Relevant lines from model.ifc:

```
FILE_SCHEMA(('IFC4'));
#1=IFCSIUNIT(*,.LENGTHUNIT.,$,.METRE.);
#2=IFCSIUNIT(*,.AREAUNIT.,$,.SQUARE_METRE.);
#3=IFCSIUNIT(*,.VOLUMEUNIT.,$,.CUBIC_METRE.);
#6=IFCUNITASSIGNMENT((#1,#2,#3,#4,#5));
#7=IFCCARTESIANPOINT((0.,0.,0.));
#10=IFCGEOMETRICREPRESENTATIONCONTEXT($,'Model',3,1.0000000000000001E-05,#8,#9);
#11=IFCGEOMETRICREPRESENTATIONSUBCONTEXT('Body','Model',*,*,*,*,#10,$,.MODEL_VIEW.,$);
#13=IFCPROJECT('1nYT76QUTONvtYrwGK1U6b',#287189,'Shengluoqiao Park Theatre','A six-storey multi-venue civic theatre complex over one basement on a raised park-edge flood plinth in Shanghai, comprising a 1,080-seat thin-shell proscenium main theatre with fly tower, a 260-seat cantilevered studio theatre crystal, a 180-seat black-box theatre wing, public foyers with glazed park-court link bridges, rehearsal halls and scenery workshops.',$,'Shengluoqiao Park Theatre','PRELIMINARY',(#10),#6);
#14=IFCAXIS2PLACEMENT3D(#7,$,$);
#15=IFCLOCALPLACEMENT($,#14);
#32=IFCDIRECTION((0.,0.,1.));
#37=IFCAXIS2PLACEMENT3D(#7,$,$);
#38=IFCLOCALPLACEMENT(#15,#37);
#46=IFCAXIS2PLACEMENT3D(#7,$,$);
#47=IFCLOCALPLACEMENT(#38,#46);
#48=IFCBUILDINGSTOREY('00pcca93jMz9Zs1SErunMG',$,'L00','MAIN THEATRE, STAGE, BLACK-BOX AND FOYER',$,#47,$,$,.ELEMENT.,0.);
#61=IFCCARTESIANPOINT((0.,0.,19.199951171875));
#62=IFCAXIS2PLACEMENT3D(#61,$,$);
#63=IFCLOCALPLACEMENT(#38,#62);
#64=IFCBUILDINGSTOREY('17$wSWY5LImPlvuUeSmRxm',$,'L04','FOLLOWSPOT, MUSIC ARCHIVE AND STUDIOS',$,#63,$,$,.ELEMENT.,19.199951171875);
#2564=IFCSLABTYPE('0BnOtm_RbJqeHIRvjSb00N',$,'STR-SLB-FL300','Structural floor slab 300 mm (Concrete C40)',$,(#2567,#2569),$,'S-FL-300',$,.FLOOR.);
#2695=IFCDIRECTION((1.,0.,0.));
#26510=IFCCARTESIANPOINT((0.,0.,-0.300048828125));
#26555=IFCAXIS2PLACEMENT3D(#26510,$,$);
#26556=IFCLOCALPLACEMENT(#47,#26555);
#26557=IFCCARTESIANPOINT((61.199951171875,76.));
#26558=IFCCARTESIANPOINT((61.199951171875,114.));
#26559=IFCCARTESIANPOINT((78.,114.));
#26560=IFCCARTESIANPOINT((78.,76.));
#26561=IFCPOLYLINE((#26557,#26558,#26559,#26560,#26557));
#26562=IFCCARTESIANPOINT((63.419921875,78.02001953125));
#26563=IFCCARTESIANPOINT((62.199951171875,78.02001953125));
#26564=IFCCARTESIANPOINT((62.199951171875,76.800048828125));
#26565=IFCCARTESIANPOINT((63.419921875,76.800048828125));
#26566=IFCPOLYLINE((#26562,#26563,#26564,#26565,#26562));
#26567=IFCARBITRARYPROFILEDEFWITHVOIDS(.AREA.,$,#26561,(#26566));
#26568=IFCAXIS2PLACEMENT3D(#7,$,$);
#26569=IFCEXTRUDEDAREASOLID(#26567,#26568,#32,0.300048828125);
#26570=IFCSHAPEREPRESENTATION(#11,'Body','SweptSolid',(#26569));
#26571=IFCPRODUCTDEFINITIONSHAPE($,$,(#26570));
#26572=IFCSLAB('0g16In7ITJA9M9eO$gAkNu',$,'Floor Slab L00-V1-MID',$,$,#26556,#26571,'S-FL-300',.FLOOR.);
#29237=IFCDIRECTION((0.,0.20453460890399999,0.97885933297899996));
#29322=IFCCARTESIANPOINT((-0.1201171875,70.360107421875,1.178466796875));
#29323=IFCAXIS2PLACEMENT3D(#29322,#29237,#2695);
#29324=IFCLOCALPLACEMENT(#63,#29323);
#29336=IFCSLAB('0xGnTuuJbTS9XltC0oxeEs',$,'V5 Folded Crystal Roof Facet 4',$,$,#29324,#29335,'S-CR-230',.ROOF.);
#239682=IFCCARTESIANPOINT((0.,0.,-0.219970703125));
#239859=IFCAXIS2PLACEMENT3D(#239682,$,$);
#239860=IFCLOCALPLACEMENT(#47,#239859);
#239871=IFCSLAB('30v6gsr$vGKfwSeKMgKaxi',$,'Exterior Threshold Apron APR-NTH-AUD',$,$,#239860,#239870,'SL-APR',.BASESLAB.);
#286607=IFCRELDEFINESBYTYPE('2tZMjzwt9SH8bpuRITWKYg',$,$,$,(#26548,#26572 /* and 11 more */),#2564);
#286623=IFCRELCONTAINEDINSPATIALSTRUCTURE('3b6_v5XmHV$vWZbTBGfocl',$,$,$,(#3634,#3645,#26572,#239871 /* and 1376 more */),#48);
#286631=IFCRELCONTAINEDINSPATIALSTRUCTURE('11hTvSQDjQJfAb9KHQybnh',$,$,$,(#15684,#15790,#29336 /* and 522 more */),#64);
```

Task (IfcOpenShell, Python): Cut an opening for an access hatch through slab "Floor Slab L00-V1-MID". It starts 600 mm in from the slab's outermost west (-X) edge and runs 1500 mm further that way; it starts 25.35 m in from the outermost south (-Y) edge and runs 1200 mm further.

```python
import numpy as np
import ifcopenshell
import ifcopenshell.api.feature
import ifcopenshell.api.geometry
import ifcopenshell.api.root
import ifcopenshell.geom
import ifcopenshell.util.placement
import ifcopenshell.util.representation
import ifcopenshell.util.shape
import ifcopenshell.util.unit

model = ifcopenshell.open("model.ifc")
unit_scale = ifcopenshell.util.unit.calculate_unit_scale(model)
settings = ifcopenshell.geom.settings()


def volume(element):
    """Net volume in cubic metres, openings subtracted."""
    shape = ifcopenshell.geom.create_shape(settings, element)
    return ifcopenshell.util.shape.get_volume(shape.geometry)


slab = model.by_id(26572)
before = volume(slab)

# Extent in the slab's own axes, in metres. The edges named are its -X and -Y sides.
slab_shape = ifcopenshell.geom.create_shape(settings, slab)
vertices = ifcopenshell.util.shape.get_vertices(slab_shape.geometry)
x_min, y_min, bottom = vertices.min(axis=0)
top = vertices[:, 2].max()

opening = ifcopenshell.api.root.create_entity(model, ifc_class="IfcOpeningElement", name="Access hatch opening", predefined_type="OPENING")
context = ifcopenshell.util.representation.get_context(model, "Model", "Body", "MODEL_VIEW")
width, depth = 1.5, 1.2
outline = [(0.0, 0.0), (width, 0.0), (width, depth), (0.0, depth), (0.0, 0.0)]
# Overshoot both faces by 50 mm so the cut is clean.
shape = ifcopenshell.api.geometry.add_slab_representation(
    model, context=context, depth=top - bottom + 0.1, polyline=outline
)
ifcopenshell.api.geometry.assign_representation(model, product=opening, representation=shape)

matrix = ifcopenshell.util.placement.get_local_placement(slab.ObjectPlacement)
matrix[:, 3] = matrix @ np.append(np.array([x_min + 0.6, y_min + 25.35, bottom - 0.05]) / unit_scale, 1.0)
ifcopenshell.api.geometry.edit_object_placement(model, product=opening, matrix=matrix, is_si=False)
ifcopenshell.api.feature.add_feature(model, feature=opening, element=slab)

after = volume(slab)

print(f"slab volume {before:.3f} -> {after:.3f} m3")

model.write("model_edited.ifc")
```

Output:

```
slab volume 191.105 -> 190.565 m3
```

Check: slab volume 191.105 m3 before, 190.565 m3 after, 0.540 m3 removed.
